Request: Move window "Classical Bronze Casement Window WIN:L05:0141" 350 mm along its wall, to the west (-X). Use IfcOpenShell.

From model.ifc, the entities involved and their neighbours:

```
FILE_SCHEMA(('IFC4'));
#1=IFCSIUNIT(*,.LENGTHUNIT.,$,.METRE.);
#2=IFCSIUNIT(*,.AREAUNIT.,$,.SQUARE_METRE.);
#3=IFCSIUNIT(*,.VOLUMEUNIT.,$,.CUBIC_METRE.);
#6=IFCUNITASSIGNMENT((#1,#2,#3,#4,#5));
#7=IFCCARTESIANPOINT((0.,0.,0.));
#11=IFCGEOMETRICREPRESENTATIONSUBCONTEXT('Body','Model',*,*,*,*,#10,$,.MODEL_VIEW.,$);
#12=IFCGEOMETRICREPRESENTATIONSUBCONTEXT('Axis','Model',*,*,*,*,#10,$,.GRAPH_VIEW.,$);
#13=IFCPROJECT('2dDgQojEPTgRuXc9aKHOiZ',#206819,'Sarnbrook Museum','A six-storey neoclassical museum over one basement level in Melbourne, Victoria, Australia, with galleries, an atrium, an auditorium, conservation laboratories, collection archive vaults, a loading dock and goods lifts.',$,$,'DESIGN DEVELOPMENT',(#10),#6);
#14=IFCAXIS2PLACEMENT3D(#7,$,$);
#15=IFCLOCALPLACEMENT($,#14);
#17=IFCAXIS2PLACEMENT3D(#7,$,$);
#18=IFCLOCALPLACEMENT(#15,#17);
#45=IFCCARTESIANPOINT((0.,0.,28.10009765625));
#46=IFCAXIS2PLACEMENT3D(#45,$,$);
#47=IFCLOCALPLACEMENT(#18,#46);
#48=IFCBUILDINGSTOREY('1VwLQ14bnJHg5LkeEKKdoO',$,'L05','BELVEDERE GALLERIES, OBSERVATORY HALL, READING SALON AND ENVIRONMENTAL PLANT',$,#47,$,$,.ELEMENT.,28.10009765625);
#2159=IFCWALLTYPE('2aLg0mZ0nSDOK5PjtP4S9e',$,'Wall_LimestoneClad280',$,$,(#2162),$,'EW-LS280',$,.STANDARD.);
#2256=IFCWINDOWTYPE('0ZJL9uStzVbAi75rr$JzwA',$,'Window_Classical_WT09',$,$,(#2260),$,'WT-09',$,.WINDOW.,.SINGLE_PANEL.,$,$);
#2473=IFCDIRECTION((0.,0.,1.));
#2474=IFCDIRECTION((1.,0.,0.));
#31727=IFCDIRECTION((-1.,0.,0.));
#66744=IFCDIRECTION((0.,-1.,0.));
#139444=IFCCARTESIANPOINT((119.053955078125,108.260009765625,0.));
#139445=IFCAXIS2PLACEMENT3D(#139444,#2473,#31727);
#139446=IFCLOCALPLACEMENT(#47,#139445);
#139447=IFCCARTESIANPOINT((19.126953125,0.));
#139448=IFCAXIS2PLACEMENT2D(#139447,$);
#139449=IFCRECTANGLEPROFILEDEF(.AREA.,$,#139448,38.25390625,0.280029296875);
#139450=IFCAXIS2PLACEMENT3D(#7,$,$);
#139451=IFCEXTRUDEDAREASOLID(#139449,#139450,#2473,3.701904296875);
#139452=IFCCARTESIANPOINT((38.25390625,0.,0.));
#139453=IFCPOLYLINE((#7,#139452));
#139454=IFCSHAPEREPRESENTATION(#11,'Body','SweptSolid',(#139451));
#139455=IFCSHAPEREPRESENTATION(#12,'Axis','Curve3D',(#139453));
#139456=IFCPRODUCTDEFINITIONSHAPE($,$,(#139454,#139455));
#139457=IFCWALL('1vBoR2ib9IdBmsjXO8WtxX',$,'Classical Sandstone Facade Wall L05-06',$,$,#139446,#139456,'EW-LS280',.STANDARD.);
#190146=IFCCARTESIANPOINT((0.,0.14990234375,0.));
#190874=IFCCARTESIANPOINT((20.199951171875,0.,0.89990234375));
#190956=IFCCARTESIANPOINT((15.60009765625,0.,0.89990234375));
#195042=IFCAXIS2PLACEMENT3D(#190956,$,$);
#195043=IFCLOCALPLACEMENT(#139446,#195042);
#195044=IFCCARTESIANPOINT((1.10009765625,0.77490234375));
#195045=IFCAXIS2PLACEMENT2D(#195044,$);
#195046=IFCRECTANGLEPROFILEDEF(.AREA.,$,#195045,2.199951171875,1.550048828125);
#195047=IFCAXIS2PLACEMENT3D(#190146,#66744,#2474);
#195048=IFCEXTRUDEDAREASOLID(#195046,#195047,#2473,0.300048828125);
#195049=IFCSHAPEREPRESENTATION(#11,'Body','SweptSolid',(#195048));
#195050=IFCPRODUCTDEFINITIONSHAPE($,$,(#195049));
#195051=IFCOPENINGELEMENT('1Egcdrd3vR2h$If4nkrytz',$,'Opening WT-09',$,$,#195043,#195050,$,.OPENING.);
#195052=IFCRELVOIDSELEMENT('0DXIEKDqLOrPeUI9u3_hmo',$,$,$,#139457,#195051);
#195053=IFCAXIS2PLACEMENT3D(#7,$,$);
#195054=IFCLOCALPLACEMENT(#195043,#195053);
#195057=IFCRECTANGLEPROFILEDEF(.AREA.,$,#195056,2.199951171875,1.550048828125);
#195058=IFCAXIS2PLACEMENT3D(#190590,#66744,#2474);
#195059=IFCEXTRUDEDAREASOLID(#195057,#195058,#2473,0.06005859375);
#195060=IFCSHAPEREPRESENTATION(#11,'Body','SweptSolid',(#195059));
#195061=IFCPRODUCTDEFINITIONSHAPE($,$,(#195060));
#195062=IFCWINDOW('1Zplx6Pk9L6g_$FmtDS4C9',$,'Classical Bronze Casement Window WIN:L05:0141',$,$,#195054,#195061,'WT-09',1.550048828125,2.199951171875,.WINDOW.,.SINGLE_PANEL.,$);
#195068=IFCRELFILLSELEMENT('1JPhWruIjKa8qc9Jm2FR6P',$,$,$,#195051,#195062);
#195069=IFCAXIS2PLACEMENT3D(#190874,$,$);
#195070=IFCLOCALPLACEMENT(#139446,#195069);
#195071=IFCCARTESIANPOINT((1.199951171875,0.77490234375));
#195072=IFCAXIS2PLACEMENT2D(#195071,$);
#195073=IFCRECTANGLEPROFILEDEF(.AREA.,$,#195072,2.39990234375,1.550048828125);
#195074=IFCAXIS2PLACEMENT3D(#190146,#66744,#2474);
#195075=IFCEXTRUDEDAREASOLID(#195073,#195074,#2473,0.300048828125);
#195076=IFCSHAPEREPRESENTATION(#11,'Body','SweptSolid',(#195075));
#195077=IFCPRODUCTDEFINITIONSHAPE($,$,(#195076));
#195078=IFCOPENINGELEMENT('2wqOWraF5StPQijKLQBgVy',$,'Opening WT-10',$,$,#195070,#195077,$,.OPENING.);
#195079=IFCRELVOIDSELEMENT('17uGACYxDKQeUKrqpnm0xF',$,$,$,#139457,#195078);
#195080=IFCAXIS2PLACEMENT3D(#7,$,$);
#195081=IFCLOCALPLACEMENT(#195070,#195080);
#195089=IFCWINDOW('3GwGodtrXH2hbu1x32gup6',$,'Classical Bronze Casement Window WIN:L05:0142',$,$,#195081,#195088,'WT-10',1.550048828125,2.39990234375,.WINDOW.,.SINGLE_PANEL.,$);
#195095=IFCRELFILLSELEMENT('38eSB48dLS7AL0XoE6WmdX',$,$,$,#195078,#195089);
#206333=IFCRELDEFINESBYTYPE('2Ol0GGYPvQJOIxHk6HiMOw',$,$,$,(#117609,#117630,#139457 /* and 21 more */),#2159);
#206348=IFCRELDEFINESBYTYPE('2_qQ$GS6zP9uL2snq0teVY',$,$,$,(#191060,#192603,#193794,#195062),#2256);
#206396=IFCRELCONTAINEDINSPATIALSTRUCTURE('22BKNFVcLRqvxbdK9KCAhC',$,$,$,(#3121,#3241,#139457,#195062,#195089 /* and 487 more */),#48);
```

```python
import ifcopenshell
import ifcopenshell.api.geometry
import ifcopenshell.util.placement

model = ifcopenshell.open("model.ifc")

window = model.by_id(195062)
opening = window.FillsVoids[0].RelatingOpeningElement
wall = opening.VoidsElements[0].RelatingBuildingElement

wall_matrix = ifcopenshell.util.placement.get_local_placement(wall.ObjectPlacement)
shift = wall_matrix[:3, 0] * 0.35
before = ifcopenshell.util.placement.get_local_placement(window.ObjectPlacement)[:3, 3].copy()

# The window is placed relative to its opening, so it follows when the opening moves.
matrix = ifcopenshell.util.placement.get_local_placement(opening.ObjectPlacement)
matrix[:3, 3] += shift
ifcopenshell.api.geometry.edit_object_placement(
    model, product=opening, matrix=matrix, is_si=False, should_transform_children=True
)

after = ifcopenshell.util.placement.get_local_placement(window.ObjectPlacement)[:3, 3]
print("window moved by", (after - before).round(3) + 0.0)

model.write("model_edited.ifc")
```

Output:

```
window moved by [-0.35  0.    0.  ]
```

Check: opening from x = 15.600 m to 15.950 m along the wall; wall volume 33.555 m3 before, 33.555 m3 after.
